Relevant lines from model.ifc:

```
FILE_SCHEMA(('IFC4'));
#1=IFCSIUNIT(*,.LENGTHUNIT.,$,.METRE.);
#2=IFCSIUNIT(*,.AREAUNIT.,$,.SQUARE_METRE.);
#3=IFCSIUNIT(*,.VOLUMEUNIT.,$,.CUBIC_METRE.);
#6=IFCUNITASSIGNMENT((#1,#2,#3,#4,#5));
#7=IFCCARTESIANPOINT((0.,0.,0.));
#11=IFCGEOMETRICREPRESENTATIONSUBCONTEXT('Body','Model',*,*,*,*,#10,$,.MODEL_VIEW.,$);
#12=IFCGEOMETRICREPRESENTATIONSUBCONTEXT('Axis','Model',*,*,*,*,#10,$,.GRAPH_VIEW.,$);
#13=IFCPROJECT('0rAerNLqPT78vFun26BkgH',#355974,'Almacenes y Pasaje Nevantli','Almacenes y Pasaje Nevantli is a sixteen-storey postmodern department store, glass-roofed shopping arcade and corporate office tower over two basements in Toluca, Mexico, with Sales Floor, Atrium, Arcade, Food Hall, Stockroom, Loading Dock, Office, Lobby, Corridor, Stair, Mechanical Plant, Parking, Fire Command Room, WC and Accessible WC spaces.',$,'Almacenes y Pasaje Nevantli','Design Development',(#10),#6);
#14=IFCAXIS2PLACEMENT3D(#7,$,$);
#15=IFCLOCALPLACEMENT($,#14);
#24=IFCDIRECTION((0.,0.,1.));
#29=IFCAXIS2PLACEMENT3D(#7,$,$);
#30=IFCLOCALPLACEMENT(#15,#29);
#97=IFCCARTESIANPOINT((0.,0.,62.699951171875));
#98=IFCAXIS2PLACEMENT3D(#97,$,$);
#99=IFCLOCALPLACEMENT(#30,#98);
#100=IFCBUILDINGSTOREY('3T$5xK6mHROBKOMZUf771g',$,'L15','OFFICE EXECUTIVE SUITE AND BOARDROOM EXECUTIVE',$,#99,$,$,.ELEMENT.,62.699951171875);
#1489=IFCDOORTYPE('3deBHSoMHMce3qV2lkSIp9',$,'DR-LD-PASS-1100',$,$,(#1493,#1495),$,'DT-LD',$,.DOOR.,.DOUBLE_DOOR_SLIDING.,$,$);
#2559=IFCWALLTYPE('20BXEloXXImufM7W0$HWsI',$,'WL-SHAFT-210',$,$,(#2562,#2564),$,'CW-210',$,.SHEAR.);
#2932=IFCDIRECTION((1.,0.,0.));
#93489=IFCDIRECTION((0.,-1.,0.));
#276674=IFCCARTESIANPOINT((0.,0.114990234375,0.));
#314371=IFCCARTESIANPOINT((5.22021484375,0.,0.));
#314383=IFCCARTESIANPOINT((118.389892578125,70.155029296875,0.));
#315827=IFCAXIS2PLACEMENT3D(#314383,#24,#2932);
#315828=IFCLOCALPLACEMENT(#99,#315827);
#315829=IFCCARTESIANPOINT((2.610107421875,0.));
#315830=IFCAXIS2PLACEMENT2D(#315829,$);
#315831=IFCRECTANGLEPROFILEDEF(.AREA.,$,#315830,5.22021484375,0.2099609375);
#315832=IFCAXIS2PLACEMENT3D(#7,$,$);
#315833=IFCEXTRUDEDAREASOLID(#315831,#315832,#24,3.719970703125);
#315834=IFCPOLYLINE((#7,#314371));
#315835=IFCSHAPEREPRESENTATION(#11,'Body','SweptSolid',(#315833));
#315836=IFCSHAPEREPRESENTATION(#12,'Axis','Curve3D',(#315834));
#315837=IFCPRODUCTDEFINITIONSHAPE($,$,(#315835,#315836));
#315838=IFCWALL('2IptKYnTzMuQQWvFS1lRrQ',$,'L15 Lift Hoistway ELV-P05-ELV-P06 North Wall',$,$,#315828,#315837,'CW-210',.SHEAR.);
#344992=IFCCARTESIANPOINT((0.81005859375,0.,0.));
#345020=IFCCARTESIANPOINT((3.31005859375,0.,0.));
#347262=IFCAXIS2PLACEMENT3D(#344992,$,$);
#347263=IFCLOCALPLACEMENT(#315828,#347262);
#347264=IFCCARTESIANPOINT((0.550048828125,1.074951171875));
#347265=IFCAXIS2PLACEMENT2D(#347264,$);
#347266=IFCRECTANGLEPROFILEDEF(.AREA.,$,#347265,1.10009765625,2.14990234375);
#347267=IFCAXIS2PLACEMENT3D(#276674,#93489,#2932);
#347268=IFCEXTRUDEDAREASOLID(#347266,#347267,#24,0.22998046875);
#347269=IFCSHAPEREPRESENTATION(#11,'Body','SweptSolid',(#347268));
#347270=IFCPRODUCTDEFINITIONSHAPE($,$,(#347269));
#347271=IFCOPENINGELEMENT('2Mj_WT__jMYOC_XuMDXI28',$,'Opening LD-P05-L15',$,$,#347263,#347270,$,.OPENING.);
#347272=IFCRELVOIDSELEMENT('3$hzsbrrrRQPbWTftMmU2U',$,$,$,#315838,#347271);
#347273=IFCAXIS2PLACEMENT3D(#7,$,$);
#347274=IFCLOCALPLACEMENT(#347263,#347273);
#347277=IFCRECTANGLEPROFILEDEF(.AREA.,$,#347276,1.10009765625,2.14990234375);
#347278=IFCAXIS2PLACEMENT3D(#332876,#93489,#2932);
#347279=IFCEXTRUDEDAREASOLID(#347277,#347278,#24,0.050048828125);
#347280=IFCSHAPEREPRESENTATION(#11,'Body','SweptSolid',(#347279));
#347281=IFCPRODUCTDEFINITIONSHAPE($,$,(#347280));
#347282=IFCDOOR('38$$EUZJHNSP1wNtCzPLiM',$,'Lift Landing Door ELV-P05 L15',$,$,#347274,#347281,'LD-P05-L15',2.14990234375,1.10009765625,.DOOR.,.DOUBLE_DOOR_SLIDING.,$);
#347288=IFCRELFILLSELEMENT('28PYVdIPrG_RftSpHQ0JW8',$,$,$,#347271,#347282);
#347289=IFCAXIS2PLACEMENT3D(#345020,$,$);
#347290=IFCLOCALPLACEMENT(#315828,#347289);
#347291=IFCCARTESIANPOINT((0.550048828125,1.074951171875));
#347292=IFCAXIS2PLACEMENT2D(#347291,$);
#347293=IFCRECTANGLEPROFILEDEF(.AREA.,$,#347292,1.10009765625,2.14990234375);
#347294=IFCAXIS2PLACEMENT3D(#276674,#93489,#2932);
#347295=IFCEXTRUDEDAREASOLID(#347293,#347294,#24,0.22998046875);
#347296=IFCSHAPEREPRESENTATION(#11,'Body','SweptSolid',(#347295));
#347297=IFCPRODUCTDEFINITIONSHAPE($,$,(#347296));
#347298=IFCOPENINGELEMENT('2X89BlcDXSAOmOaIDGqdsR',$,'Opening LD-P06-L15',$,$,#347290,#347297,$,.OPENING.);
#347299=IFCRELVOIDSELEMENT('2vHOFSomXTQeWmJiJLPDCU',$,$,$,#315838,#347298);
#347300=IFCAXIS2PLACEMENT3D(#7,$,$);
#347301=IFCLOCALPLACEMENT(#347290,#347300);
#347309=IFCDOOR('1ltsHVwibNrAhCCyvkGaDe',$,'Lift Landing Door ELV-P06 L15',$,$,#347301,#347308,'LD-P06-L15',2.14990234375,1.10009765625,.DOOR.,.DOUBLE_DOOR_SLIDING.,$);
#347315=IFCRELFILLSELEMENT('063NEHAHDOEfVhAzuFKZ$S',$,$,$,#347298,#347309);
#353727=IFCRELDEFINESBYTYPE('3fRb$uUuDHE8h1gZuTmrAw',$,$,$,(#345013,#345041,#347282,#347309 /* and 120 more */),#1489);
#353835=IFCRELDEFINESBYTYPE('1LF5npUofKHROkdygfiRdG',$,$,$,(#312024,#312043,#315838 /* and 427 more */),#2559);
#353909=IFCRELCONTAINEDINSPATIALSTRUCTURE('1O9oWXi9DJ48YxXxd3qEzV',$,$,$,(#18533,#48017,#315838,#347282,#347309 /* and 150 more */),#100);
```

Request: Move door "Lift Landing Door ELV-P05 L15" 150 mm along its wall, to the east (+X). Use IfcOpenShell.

```python
import ifcopenshell
import ifcopenshell.api.geometry
import ifcopenshell.util.placement
import ifcopenshell.util.unit

model = ifcopenshell.open("model.ifc")
unit_scale = ifcopenshell.util.unit.calculate_unit_scale(model)

door = model.by_guid("38$$EUZJHNSP1wNtCzPLiM")
opening = door.FillsVoids[0].RelatingOpeningElement
wall = opening.VoidsElements[0].RelatingBuildingElement

wall_matrix = ifcopenshell.util.placement.get_local_placement(wall.ObjectPlacement)
shift = wall_matrix[:3, 0] * 0.15 / unit_scale
before = ifcopenshell.util.placement.get_local_placement(door.ObjectPlacement)[:3, 3].copy()

# The door is placed relative to its opening, so it follows when the opening moves.
matrix = ifcopenshell.util.placement.get_local_placement(opening.ObjectPlacement)
matrix[:3, 3] += shift
ifcopenshell.api.geometry.edit_object_placement(
    model, product=opening, matrix=matrix, is_si=False, should_transform_children=True
)

after = ifcopenshell.util.placement.get_local_placement(door.ObjectPlacement)[:3, 3]
print("door moved by", (after - before).round(3) + 0.0)

model.write("model_rev.ifc")
```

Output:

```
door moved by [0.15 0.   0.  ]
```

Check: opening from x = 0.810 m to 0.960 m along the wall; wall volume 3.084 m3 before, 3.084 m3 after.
